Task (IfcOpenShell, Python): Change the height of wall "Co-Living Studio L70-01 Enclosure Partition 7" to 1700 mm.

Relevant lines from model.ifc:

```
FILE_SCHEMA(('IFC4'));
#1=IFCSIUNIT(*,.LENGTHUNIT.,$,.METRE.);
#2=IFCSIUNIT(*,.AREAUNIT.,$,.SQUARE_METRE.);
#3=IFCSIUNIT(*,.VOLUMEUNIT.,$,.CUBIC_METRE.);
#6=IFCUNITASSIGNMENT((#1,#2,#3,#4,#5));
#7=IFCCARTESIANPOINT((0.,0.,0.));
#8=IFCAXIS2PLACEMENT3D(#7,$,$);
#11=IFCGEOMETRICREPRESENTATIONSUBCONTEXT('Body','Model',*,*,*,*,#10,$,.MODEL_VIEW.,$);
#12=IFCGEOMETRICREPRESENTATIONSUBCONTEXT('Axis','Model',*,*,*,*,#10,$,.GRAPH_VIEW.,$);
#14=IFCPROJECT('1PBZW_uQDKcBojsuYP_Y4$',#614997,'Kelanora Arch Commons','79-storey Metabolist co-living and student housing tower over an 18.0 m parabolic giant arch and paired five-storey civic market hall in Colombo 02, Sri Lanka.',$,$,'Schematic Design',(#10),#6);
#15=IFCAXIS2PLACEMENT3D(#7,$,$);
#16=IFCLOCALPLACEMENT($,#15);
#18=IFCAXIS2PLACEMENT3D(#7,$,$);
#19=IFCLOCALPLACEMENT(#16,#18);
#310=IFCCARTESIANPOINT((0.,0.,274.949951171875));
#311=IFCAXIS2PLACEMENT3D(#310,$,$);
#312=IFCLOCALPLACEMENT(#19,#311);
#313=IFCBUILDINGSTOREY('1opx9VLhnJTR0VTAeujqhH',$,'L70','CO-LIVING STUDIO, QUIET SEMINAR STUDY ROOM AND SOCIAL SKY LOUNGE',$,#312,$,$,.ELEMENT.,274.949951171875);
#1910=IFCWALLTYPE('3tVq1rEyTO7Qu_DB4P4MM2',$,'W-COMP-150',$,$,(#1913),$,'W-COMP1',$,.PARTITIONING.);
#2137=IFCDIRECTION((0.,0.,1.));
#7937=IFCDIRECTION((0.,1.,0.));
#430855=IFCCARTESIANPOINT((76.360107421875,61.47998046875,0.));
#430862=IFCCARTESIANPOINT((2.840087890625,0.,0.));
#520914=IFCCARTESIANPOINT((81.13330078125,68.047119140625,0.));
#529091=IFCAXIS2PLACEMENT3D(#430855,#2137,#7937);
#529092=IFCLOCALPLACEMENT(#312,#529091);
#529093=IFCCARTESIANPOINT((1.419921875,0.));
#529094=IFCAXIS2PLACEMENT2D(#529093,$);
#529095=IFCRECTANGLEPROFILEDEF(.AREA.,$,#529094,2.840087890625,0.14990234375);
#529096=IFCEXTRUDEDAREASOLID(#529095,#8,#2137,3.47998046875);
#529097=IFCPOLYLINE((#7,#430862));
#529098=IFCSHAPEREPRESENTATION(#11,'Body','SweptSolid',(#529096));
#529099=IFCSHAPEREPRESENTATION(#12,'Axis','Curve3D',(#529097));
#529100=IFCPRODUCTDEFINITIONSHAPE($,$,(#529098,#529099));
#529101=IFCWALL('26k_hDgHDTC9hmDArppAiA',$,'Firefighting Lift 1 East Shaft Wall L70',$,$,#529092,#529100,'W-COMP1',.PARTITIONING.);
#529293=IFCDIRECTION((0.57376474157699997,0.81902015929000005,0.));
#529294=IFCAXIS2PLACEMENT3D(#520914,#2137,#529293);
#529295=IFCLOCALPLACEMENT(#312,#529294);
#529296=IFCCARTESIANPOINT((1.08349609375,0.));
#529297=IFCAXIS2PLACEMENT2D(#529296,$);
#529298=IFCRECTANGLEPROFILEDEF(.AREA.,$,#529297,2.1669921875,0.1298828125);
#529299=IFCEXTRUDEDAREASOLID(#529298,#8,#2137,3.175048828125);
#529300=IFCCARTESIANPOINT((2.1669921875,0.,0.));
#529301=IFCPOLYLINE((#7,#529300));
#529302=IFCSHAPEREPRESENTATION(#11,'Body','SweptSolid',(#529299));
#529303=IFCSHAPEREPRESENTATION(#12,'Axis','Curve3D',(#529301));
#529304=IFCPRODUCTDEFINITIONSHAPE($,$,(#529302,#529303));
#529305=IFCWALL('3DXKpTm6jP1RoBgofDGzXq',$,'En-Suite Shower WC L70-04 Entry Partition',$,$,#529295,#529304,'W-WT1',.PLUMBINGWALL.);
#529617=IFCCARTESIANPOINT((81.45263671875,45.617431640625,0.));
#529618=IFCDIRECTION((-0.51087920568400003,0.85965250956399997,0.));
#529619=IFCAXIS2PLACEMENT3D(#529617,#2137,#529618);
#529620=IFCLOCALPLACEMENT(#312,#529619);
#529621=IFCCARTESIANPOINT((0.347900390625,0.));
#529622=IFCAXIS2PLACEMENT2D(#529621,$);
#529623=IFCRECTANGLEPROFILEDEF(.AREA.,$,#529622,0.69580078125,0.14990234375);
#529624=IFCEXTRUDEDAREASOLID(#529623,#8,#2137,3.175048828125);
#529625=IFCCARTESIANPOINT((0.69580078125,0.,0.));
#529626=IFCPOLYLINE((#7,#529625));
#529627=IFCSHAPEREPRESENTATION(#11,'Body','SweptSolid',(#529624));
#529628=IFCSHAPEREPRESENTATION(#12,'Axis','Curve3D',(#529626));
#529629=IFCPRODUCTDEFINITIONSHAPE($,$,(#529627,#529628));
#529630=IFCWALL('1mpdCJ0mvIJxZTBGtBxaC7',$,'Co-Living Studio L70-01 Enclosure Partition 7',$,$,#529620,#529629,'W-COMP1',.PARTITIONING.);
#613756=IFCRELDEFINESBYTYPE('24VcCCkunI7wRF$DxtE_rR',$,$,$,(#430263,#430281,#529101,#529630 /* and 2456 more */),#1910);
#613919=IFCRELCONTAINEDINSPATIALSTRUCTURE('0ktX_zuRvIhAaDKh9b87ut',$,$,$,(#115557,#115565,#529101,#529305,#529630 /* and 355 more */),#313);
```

```python
import ifcopenshell
import ifcopenshell.geom
import ifcopenshell.util.representation
import ifcopenshell.util.shape

model = ifcopenshell.open("model.ifc")
settings = ifcopenshell.geom.settings()


def volume(element):
    """Net volume in cubic metres, openings subtracted."""
    shape = ifcopenshell.geom.create_shape(settings, element)
    return ifcopenshell.util.shape.get_volume(shape.geometry)


wall = model.by_guid("1mpdCJ0mvIJxZTBGtBxaC7")
before = volume(wall)

body = ifcopenshell.util.representation.get_representation(wall, "Model", "Body")
solid = body.Items[0]
old_height = solid.Depth
solid.Depth = 1.7
after = volume(wall)

print(f"height {old_height:g} -> {solid.Depth:g}, volume {before:.3f} -> {after:.3f} m3")

model.write("model_rev.ifc")
```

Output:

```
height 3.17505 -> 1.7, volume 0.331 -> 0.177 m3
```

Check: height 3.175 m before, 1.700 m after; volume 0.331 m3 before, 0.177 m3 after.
